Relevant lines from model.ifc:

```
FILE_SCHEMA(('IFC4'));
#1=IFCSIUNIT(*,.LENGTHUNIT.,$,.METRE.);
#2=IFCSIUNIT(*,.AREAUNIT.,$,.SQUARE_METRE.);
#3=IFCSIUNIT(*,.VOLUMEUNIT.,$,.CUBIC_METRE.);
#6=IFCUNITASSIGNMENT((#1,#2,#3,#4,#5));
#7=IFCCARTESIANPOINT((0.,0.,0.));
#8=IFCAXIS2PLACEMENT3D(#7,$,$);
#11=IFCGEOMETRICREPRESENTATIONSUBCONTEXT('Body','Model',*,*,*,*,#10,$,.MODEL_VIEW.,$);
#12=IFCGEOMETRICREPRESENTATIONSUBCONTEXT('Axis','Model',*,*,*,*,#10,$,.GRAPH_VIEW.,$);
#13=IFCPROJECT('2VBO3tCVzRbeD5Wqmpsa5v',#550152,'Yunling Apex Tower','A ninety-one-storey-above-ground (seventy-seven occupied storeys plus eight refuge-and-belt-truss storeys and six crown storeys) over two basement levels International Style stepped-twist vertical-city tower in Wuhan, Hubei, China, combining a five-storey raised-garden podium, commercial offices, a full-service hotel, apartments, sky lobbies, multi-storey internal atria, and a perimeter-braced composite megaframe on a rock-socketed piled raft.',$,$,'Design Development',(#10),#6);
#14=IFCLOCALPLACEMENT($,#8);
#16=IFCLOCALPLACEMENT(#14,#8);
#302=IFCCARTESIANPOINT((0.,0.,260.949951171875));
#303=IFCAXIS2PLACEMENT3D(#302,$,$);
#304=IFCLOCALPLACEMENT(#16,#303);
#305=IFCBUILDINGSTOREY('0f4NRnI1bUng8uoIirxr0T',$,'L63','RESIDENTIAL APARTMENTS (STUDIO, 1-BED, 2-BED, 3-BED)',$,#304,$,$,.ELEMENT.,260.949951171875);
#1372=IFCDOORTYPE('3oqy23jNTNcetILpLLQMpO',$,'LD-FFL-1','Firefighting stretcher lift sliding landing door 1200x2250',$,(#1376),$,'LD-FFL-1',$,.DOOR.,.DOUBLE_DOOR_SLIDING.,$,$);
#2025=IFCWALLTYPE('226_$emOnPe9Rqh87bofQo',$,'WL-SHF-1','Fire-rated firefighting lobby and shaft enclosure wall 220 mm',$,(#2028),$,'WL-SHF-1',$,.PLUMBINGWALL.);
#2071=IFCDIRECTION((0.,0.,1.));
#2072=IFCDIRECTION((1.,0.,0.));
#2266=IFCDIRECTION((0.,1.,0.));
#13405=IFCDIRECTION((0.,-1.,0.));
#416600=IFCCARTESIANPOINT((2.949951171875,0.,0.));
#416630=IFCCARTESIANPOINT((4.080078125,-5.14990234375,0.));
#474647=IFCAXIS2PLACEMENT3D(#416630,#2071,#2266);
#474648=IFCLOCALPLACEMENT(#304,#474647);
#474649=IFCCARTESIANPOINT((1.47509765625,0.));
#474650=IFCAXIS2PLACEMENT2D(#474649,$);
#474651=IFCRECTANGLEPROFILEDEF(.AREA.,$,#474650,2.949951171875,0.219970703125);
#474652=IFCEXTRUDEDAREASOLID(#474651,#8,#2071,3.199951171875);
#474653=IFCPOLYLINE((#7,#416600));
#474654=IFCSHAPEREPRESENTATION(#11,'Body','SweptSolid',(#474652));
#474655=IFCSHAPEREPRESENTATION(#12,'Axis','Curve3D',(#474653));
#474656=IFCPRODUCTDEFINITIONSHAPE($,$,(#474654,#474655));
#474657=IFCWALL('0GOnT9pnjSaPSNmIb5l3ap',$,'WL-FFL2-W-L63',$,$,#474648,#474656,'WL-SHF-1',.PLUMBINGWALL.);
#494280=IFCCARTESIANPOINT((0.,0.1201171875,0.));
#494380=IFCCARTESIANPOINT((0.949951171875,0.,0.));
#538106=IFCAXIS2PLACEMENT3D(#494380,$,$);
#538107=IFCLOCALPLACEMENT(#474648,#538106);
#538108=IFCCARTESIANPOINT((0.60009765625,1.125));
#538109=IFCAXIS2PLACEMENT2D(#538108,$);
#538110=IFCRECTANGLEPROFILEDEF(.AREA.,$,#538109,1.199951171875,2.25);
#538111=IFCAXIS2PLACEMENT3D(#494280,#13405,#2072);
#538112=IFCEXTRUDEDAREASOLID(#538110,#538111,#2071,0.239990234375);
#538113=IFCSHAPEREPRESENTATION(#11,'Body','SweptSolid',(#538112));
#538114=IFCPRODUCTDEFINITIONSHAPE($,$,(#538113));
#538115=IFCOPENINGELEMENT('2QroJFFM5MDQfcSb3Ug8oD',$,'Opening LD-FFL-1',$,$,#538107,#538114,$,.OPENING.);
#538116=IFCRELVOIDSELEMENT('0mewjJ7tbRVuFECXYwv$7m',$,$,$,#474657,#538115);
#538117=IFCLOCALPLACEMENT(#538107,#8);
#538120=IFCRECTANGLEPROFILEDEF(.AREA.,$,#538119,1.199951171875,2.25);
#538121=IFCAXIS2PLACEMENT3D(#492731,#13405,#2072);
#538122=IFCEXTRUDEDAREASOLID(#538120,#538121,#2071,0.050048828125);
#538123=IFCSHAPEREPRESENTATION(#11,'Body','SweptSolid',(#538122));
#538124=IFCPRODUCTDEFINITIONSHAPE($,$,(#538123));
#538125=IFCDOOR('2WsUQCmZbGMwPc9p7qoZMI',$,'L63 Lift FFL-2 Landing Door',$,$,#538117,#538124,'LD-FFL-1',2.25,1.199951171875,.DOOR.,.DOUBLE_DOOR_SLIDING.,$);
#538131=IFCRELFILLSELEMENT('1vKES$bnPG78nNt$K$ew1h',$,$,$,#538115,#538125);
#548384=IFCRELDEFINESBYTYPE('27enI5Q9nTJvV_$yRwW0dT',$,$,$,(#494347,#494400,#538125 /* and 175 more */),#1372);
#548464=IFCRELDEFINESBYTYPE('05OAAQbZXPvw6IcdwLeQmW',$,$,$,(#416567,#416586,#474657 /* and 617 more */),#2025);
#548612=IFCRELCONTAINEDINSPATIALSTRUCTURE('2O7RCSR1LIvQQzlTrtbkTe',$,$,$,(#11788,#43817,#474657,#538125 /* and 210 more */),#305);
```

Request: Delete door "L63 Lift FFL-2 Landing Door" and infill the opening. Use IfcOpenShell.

```python
import ifcopenshell
import ifcopenshell.api.feature
import ifcopenshell.api.root
import ifcopenshell.geom
import ifcopenshell.util.shape

model = ifcopenshell.open("model.ifc")
settings = ifcopenshell.geom.settings()


def volume(element):
    """Net volume in cubic metres, openings subtracted."""
    shape = ifcopenshell.geom.create_shape(settings, element)
    return ifcopenshell.util.shape.get_volume(shape.geometry)


door = model.by_guid("2WsUQCmZbGMwPc9p7qoZMI")
opening = door.FillsVoids[0].RelatingOpeningElement
wall = opening.VoidsElements[0].RelatingBuildingElement
before = volume(wall)

ifcopenshell.api.root.remove_product(model, product=door)
ifcopenshell.api.feature.remove_feature(model, feature=opening)

after = volume(wall)

print(f"wall volume {before:.3f} -> {after:.3f} m3")

model.write("model_updated.ifc")
```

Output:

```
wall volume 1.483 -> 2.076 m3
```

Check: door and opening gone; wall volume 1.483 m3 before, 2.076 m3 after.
